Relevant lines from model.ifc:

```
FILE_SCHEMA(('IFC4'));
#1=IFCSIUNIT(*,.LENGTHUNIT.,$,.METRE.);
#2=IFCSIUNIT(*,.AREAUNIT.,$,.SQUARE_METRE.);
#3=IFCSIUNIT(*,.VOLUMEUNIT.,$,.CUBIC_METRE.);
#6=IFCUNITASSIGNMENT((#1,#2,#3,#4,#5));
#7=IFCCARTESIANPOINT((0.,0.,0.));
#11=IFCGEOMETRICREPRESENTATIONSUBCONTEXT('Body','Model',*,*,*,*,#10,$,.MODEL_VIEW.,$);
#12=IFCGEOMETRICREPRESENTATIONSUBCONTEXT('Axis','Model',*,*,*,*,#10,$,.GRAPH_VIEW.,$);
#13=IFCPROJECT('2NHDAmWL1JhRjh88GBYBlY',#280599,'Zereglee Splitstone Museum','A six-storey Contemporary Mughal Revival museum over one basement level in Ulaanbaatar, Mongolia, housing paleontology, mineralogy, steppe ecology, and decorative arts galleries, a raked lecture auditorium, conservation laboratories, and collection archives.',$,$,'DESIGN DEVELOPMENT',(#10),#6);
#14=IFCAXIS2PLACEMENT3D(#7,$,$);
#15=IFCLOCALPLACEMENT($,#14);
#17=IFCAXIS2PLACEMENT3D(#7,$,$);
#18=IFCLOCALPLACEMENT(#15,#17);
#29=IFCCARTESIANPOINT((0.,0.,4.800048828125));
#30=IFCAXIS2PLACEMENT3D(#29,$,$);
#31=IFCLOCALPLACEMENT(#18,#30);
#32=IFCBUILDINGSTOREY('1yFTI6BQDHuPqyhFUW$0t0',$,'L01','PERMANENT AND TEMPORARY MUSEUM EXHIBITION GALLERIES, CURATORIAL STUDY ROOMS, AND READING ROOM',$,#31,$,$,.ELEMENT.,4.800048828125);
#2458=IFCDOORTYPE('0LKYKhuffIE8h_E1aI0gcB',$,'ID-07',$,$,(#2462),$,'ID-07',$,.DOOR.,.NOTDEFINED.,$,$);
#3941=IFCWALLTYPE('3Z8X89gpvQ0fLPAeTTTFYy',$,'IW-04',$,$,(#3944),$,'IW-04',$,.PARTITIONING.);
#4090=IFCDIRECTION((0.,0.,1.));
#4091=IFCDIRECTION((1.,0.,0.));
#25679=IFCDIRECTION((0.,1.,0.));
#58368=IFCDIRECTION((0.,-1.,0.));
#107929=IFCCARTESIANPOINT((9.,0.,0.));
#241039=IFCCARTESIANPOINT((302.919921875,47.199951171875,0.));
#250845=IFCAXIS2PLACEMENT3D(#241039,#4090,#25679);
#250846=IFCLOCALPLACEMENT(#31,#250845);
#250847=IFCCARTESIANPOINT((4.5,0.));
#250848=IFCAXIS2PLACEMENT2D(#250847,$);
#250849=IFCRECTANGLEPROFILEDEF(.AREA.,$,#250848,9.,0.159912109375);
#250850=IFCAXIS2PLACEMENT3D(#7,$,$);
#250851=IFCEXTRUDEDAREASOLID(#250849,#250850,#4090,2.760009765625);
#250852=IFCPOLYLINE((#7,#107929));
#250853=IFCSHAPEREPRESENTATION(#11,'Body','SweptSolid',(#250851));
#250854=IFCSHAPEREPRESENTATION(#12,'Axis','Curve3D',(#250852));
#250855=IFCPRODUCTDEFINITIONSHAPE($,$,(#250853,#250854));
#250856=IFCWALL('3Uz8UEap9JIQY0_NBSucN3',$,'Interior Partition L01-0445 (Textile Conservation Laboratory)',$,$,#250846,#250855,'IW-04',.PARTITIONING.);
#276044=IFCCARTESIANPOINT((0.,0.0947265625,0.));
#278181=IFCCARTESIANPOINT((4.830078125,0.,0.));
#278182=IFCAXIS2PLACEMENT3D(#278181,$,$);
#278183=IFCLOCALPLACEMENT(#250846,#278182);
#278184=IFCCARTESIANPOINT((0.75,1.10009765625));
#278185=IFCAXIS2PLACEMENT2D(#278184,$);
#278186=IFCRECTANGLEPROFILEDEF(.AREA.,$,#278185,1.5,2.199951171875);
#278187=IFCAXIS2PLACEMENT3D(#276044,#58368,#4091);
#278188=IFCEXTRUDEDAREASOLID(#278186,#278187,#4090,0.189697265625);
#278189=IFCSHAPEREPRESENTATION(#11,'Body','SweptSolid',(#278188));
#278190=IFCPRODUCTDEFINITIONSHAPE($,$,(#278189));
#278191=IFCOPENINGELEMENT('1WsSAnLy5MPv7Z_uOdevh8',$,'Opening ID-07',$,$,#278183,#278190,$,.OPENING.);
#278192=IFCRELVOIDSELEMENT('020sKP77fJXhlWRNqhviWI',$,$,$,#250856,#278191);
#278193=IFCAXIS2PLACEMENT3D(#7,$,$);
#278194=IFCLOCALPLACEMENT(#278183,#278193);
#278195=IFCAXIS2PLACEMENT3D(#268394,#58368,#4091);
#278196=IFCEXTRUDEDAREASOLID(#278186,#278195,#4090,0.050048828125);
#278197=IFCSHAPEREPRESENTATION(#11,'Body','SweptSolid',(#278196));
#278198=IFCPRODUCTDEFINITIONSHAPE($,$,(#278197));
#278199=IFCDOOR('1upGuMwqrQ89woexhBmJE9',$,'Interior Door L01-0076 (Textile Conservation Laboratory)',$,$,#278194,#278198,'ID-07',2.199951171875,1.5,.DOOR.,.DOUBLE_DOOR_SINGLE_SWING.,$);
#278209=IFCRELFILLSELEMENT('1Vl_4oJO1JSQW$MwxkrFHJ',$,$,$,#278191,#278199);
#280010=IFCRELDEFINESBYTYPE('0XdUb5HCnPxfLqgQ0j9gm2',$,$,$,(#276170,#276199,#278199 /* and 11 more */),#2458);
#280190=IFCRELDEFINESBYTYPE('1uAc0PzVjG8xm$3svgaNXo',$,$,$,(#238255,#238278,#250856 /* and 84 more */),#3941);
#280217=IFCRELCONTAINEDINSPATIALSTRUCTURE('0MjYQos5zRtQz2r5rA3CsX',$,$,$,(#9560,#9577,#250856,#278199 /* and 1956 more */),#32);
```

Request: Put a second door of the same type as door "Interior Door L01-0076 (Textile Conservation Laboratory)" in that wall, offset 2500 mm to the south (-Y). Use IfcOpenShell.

```python
import ifcopenshell
import ifcopenshell.api.feature
import ifcopenshell.api.geometry
import ifcopenshell.api.root
import ifcopenshell.geom
import ifcopenshell.util.element
import ifcopenshell.util.placement
import ifcopenshell.util.shape
import ifcopenshell.util.unit

model = ifcopenshell.open("model.ifc")
unit_scale = ifcopenshell.util.unit.calculate_unit_scale(model)
settings = ifcopenshell.geom.settings()


def volume(element):
    """Net volume in cubic metres, openings subtracted."""
    shape = ifcopenshell.geom.create_shape(settings, element)
    return ifcopenshell.util.shape.get_volume(shape.geometry)


door = model.by_guid("1upGuMwqrQ89woexhBmJE9")
opening = door.FillsVoids[0].RelatingOpeningElement
wall = opening.VoidsElements[0].RelatingBuildingElement
before = volume(wall)
shift = ifcopenshell.util.placement.get_local_placement(wall.ObjectPlacement)[:3, 0] * -2.5 / unit_scale

# copy_class copies the void relationship, type, container and properties, but no geometry.
new_opening = ifcopenshell.api.root.copy_class(model, product=opening)
new_opening.Representation = ifcopenshell.util.element.copy_deep(
    model, opening.Representation, exclude=["IfcGeometricRepresentationContext", "IfcRepresentationMap"]
)
new_door = ifcopenshell.api.root.copy_class(model, product=door)
new_door.Representation = ifcopenshell.util.element.copy_deep(
    model, door.Representation, exclude=["IfcGeometricRepresentationContext", "IfcRepresentationMap"]
)
new_door.Tag = None
ifcopenshell.api.feature.add_filling(model, opening=new_opening, element=new_door)

for old, new in ((opening, new_opening), (door, new_door)):
    matrix = ifcopenshell.util.placement.get_local_placement(old.ObjectPlacement)
    matrix[:3, 3] += shift
    ifcopenshell.api.geometry.edit_object_placement(model, product=new, matrix=matrix, is_si=False)

after = volume(wall)

print(f"wall volume {before:.3f} -> {after:.3f} m3")

model.write("model_updated.ifc")
```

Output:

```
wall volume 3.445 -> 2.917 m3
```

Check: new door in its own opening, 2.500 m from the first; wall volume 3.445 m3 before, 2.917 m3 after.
